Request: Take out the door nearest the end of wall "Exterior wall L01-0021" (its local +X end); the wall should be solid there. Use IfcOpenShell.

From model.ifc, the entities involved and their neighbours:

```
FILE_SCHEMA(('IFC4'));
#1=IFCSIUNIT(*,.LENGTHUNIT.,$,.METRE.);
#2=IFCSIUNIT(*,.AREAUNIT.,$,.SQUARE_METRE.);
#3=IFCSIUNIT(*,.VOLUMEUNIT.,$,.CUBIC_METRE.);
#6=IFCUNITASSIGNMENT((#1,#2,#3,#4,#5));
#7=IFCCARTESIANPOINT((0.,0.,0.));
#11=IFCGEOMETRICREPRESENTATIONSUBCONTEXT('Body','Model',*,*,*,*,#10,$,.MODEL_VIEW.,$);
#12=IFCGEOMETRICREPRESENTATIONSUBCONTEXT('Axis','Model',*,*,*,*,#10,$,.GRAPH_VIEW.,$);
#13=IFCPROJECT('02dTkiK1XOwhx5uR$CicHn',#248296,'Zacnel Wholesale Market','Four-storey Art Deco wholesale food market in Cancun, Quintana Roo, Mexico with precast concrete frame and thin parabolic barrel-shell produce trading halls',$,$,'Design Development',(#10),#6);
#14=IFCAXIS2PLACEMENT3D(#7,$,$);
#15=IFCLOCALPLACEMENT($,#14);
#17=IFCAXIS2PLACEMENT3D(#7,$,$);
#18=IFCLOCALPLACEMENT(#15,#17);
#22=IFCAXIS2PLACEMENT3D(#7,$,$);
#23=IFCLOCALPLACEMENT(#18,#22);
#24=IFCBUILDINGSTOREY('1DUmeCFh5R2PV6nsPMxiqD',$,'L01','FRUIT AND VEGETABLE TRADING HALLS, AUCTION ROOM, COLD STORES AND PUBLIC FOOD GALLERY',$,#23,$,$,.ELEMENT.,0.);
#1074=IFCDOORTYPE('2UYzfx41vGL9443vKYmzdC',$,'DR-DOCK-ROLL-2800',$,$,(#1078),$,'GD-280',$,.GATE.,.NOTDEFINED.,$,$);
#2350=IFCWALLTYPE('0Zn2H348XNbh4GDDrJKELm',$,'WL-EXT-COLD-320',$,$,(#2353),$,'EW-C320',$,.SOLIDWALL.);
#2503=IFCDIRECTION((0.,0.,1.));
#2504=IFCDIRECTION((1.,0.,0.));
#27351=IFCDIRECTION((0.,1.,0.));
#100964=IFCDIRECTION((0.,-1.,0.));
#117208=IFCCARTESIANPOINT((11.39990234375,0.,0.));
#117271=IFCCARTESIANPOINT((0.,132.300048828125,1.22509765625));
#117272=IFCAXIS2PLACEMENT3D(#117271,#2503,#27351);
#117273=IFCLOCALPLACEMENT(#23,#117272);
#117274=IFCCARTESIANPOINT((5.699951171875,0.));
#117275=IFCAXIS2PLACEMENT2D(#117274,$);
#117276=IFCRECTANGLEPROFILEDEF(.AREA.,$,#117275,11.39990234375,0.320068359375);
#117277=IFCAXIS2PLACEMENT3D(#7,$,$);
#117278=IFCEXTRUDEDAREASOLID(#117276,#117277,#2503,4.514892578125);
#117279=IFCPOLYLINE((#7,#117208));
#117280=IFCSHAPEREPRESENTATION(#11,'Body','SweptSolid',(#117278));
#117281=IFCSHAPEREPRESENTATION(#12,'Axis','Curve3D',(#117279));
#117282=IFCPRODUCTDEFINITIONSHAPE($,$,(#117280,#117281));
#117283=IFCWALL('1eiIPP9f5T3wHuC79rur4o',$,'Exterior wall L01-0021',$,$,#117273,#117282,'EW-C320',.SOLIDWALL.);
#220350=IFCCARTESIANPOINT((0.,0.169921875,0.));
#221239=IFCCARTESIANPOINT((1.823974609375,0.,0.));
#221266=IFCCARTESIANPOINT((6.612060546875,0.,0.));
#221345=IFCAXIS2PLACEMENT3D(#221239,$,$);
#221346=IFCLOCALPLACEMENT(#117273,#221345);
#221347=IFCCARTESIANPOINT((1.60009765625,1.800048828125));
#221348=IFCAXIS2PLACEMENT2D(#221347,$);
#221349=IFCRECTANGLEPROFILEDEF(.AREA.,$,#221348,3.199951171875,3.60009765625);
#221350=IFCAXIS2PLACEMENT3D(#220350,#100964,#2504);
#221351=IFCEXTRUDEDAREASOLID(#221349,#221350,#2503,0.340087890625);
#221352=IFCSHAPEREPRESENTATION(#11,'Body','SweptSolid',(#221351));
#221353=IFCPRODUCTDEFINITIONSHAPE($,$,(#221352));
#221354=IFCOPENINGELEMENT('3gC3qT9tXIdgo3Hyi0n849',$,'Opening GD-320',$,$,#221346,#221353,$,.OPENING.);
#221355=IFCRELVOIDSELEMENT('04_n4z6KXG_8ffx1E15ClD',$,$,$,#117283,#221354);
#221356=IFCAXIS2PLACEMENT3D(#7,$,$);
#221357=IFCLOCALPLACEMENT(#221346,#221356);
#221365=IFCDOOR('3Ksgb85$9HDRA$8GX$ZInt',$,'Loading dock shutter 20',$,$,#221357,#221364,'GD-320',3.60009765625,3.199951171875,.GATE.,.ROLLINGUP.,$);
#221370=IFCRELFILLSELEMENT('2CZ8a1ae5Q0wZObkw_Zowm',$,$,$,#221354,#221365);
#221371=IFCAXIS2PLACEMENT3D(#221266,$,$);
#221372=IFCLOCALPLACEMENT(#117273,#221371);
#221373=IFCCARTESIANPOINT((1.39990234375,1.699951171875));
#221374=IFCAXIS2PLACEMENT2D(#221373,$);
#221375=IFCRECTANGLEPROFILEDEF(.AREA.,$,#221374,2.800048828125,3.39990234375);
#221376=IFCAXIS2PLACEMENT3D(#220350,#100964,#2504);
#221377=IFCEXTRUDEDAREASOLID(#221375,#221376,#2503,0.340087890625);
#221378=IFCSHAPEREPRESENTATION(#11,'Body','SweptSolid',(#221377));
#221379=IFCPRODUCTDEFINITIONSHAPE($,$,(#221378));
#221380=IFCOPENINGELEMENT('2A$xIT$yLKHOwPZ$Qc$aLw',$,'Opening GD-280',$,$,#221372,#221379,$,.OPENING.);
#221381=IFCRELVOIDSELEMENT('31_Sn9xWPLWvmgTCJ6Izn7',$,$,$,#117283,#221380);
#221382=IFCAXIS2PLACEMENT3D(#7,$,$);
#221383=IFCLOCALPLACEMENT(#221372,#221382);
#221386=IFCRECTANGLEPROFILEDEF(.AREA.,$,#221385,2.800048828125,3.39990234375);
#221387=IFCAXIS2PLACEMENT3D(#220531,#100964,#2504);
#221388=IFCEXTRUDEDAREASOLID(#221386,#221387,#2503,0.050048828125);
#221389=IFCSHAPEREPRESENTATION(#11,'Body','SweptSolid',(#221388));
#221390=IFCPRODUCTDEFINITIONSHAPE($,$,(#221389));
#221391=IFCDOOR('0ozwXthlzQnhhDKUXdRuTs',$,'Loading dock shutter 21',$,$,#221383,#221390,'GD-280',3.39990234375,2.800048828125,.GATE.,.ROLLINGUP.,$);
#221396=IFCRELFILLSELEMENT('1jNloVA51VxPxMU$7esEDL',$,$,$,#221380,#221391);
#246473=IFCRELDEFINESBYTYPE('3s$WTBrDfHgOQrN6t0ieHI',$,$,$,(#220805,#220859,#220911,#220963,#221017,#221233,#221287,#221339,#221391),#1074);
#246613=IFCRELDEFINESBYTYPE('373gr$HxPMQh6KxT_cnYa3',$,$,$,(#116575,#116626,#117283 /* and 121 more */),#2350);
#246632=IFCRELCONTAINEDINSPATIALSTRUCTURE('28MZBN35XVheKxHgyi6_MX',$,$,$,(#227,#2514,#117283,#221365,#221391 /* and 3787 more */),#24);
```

```python
import ifcopenshell
import ifcopenshell.api.feature
import ifcopenshell.api.root
import ifcopenshell.geom
import ifcopenshell.util.shape

model = ifcopenshell.open("model.ifc")
settings = ifcopenshell.geom.settings()


def volume(element):
    """Net volume in cubic metres, openings subtracted."""
    shape = ifcopenshell.geom.create_shape(settings, element)
    return ifcopenshell.util.shape.get_volume(shape.geometry)


door = model.by_guid("0ozwXthlzQnhhDKUXdRuTs")
opening = door.FillsVoids[0].RelatingOpeningElement
wall = opening.VoidsElements[0].RelatingBuildingElement
before = volume(wall)

ifcopenshell.api.root.remove_product(model, product=door)
ifcopenshell.api.feature.remove_feature(model, feature=opening)

after = volume(wall)

print(f"wall volume {before:.3f} -> {after:.3f} m3")

model.write("model_edited.ifc")
```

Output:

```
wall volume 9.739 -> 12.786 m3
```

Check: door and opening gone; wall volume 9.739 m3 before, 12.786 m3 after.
